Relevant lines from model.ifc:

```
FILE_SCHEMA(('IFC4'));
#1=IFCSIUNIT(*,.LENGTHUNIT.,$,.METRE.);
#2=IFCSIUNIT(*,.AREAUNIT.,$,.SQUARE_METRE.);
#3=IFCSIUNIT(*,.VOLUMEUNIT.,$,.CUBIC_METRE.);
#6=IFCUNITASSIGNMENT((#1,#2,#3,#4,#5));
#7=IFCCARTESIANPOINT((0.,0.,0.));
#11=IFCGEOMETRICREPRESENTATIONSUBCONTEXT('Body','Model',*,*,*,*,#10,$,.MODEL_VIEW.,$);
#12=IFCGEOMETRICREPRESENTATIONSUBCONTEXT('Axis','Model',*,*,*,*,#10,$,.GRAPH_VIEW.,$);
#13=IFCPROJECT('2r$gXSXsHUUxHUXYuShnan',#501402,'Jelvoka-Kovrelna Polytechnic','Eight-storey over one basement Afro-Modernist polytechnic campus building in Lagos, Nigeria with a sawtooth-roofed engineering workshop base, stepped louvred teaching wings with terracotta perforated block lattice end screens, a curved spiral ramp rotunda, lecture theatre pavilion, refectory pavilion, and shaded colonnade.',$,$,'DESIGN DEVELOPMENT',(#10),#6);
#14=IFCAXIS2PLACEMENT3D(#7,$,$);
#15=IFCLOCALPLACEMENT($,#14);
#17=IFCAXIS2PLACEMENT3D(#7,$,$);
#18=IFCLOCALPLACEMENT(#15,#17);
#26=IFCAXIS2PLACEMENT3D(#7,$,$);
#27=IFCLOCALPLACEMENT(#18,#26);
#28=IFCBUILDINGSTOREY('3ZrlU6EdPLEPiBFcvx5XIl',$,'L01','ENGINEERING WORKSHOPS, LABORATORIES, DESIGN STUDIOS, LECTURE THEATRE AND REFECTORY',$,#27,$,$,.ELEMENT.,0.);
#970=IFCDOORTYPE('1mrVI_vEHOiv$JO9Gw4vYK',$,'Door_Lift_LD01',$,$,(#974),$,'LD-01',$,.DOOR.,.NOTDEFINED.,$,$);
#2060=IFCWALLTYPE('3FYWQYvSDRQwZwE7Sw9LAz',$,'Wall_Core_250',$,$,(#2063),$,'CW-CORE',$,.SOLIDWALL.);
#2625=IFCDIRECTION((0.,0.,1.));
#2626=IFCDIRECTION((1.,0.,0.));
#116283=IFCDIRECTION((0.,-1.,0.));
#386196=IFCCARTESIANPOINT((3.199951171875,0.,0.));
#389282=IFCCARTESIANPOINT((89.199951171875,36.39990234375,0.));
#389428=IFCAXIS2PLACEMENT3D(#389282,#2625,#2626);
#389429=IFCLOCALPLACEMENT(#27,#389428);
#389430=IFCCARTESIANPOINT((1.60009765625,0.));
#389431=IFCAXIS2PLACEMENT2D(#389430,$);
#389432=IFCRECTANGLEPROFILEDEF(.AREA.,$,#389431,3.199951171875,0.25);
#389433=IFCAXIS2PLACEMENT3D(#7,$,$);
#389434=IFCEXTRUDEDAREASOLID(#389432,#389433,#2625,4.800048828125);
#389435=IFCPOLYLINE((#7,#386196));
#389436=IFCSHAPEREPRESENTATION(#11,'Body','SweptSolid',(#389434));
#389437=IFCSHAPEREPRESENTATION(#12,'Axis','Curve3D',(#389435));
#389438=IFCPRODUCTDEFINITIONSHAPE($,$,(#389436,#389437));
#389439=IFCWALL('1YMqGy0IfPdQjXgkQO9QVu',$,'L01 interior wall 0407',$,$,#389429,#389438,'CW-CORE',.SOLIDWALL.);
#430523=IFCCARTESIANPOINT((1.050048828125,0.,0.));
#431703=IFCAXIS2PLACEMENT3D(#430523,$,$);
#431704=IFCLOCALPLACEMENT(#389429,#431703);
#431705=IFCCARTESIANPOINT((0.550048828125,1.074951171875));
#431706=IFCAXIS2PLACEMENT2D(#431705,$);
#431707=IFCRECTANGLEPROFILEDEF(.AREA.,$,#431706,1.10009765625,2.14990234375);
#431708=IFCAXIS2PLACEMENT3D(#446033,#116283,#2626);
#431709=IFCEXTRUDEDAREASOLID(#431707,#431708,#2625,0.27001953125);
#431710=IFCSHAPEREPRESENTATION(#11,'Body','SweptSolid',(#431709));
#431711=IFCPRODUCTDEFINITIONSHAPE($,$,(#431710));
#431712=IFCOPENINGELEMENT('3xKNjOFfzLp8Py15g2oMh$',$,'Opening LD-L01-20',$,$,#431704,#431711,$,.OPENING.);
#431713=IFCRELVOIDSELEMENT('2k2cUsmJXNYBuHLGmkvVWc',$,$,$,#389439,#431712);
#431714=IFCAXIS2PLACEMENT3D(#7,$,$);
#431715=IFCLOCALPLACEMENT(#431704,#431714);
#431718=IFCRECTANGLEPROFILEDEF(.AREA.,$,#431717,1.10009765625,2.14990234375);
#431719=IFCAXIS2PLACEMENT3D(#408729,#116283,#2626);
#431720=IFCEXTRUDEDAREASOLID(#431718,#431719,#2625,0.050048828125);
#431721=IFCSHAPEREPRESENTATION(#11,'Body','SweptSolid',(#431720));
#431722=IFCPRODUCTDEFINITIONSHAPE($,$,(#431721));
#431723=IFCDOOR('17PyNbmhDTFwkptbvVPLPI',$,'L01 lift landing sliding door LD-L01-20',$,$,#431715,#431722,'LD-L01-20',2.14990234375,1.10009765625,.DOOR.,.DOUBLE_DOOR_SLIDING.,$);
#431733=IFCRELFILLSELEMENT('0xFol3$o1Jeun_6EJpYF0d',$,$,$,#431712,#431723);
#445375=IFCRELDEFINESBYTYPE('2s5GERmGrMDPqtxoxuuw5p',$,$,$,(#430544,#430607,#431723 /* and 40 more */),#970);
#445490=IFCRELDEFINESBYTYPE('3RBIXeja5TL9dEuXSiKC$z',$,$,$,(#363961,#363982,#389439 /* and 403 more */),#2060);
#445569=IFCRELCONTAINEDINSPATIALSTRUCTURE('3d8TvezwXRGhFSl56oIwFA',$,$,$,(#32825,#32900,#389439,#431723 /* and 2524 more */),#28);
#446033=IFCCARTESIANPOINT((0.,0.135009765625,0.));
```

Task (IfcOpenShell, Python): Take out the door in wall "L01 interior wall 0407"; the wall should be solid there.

```python
import ifcopenshell
import ifcopenshell.api.feature
import ifcopenshell.api.root
import ifcopenshell.geom
import ifcopenshell.util.shape

model = ifcopenshell.open("model.ifc")
settings = ifcopenshell.geom.settings()


def volume(element):
    """Net volume in cubic metres, openings subtracted."""
    shape = ifcopenshell.geom.create_shape(settings, element)
    return ifcopenshell.util.shape.get_volume(shape.geometry)


door = model.by_id(431723)
opening = door.FillsVoids[0].RelatingOpeningElement
wall = opening.VoidsElements[0].RelatingBuildingElement
before = volume(wall)

ifcopenshell.api.root.remove_product(model, product=door)
ifcopenshell.api.feature.remove_feature(model, feature=opening)

after = volume(wall)

print(f"wall volume {before:.3f} -> {after:.3f} m3")

model.write("model-out.ifc")
```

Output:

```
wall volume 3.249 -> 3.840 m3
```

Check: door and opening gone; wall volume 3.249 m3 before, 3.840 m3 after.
